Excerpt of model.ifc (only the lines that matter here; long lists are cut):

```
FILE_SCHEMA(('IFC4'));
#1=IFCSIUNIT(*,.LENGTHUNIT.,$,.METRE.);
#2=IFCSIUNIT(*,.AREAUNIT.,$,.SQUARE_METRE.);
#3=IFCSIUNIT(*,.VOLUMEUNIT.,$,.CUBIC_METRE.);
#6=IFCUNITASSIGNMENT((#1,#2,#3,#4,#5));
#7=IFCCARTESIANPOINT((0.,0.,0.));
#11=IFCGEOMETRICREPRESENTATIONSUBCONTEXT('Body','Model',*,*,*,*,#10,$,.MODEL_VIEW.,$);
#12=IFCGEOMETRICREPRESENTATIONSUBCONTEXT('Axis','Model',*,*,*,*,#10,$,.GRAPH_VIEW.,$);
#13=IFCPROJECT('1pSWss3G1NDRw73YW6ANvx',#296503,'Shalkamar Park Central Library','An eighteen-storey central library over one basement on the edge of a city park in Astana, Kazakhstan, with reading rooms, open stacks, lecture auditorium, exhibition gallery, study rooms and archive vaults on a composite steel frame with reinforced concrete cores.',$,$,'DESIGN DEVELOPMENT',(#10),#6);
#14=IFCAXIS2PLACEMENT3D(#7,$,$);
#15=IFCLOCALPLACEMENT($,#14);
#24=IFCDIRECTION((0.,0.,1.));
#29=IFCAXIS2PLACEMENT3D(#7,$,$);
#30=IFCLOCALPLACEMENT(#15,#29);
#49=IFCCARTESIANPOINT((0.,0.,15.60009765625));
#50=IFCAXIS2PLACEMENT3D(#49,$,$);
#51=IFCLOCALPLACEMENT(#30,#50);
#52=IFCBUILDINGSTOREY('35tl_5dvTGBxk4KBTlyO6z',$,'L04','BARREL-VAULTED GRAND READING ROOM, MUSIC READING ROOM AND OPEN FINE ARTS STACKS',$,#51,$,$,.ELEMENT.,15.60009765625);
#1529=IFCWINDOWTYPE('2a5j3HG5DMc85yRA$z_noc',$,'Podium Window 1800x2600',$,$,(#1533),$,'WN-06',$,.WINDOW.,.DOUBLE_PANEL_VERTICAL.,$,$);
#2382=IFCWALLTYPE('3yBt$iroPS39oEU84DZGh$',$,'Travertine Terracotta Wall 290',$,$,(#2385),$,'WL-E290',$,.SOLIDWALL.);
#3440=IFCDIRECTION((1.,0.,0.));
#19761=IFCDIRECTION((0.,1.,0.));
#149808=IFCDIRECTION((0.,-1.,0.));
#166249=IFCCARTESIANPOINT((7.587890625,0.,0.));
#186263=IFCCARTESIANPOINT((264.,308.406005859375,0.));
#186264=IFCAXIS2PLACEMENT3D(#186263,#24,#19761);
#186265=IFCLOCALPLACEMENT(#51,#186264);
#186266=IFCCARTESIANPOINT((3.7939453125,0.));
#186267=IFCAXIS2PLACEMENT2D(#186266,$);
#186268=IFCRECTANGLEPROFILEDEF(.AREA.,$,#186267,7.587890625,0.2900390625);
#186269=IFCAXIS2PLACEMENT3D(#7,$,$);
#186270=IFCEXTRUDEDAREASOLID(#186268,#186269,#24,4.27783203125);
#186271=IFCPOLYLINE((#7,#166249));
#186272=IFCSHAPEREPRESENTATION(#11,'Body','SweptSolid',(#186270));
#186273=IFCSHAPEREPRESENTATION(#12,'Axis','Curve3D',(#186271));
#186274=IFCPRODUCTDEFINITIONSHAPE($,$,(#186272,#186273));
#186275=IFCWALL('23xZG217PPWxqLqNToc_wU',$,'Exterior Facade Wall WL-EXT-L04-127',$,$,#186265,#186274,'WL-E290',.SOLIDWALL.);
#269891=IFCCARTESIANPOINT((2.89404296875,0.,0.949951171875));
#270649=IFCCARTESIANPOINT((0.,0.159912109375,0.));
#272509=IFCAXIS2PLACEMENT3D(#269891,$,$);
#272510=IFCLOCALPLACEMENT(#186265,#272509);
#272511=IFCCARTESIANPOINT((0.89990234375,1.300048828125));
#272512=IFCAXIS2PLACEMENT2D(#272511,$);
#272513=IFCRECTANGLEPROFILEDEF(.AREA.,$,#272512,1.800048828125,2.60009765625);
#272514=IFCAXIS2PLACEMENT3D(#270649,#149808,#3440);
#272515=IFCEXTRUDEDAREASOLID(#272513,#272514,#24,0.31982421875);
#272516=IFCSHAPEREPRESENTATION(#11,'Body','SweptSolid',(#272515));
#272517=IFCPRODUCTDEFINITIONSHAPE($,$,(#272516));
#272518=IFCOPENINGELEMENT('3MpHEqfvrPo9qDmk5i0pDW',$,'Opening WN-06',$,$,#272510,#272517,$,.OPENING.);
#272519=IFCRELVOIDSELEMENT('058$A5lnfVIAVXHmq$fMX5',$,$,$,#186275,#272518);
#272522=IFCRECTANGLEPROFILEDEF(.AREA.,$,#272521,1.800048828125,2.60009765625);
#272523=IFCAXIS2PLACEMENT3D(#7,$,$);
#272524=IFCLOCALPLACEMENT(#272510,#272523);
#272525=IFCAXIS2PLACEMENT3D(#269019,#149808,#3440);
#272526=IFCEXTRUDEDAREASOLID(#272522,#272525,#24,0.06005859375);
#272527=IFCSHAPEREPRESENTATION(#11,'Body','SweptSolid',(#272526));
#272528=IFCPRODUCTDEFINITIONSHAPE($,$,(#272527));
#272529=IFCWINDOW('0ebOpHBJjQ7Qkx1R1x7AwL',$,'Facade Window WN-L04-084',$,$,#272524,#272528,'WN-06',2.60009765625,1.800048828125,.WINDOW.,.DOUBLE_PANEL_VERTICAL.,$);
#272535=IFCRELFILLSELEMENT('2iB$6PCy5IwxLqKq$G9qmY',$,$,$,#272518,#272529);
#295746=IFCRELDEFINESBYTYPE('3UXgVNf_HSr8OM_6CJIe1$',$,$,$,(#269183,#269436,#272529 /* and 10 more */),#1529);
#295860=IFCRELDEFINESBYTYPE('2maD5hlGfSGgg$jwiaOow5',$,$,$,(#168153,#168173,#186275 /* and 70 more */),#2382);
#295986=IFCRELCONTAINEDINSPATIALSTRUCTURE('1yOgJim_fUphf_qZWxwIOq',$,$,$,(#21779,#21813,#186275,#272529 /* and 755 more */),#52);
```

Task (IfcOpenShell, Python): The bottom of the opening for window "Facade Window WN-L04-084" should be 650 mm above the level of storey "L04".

```python
import numpy as np
import ifcopenshell
import ifcopenshell.api.geometry
import ifcopenshell.geom
import ifcopenshell.util.element
import ifcopenshell.util.placement
import ifcopenshell.util.shape
import ifcopenshell.util.unit

model = ifcopenshell.open("model.ifc")
unit_scale = ifcopenshell.util.unit.calculate_unit_scale(model)

window = model.by_guid("0ebOpHBJjQ7Qkx1R1x7AwL")
opening = window.FillsVoids[0].RelatingOpeningElement
storey = ifcopenshell.util.element.get_container(window, ifc_class="IfcBuildingStorey")
level = ifcopenshell.util.placement.get_local_placement(storey.ObjectPlacement)[2, 3]

# The opening's origin need not be at the sill, so measure its lowest point.
shape = ifcopenshell.geom.create_shape(ifcopenshell.geom.settings(), opening)
bottom = ifcopenshell.util.shape.get_shape_bottom_elevation(shape, shape.geometry) / unit_scale
dz = level + 0.65 / unit_scale - bottom

shift = np.array([0.0, 0.0, dz])
# The window is placed relative to its opening, so it follows when the opening moves.
matrix = ifcopenshell.util.placement.get_local_placement(opening.ObjectPlacement)
matrix[:3, 3] += shift
ifcopenshell.api.geometry.edit_object_placement(
    model, product=opening, matrix=matrix, is_si=False, should_transform_children=True
)

print(f"moved by {dz * unit_scale:+.3f} m")

model.write("model_updated.ifc")
```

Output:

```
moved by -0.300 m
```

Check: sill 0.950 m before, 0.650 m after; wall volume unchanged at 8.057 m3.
